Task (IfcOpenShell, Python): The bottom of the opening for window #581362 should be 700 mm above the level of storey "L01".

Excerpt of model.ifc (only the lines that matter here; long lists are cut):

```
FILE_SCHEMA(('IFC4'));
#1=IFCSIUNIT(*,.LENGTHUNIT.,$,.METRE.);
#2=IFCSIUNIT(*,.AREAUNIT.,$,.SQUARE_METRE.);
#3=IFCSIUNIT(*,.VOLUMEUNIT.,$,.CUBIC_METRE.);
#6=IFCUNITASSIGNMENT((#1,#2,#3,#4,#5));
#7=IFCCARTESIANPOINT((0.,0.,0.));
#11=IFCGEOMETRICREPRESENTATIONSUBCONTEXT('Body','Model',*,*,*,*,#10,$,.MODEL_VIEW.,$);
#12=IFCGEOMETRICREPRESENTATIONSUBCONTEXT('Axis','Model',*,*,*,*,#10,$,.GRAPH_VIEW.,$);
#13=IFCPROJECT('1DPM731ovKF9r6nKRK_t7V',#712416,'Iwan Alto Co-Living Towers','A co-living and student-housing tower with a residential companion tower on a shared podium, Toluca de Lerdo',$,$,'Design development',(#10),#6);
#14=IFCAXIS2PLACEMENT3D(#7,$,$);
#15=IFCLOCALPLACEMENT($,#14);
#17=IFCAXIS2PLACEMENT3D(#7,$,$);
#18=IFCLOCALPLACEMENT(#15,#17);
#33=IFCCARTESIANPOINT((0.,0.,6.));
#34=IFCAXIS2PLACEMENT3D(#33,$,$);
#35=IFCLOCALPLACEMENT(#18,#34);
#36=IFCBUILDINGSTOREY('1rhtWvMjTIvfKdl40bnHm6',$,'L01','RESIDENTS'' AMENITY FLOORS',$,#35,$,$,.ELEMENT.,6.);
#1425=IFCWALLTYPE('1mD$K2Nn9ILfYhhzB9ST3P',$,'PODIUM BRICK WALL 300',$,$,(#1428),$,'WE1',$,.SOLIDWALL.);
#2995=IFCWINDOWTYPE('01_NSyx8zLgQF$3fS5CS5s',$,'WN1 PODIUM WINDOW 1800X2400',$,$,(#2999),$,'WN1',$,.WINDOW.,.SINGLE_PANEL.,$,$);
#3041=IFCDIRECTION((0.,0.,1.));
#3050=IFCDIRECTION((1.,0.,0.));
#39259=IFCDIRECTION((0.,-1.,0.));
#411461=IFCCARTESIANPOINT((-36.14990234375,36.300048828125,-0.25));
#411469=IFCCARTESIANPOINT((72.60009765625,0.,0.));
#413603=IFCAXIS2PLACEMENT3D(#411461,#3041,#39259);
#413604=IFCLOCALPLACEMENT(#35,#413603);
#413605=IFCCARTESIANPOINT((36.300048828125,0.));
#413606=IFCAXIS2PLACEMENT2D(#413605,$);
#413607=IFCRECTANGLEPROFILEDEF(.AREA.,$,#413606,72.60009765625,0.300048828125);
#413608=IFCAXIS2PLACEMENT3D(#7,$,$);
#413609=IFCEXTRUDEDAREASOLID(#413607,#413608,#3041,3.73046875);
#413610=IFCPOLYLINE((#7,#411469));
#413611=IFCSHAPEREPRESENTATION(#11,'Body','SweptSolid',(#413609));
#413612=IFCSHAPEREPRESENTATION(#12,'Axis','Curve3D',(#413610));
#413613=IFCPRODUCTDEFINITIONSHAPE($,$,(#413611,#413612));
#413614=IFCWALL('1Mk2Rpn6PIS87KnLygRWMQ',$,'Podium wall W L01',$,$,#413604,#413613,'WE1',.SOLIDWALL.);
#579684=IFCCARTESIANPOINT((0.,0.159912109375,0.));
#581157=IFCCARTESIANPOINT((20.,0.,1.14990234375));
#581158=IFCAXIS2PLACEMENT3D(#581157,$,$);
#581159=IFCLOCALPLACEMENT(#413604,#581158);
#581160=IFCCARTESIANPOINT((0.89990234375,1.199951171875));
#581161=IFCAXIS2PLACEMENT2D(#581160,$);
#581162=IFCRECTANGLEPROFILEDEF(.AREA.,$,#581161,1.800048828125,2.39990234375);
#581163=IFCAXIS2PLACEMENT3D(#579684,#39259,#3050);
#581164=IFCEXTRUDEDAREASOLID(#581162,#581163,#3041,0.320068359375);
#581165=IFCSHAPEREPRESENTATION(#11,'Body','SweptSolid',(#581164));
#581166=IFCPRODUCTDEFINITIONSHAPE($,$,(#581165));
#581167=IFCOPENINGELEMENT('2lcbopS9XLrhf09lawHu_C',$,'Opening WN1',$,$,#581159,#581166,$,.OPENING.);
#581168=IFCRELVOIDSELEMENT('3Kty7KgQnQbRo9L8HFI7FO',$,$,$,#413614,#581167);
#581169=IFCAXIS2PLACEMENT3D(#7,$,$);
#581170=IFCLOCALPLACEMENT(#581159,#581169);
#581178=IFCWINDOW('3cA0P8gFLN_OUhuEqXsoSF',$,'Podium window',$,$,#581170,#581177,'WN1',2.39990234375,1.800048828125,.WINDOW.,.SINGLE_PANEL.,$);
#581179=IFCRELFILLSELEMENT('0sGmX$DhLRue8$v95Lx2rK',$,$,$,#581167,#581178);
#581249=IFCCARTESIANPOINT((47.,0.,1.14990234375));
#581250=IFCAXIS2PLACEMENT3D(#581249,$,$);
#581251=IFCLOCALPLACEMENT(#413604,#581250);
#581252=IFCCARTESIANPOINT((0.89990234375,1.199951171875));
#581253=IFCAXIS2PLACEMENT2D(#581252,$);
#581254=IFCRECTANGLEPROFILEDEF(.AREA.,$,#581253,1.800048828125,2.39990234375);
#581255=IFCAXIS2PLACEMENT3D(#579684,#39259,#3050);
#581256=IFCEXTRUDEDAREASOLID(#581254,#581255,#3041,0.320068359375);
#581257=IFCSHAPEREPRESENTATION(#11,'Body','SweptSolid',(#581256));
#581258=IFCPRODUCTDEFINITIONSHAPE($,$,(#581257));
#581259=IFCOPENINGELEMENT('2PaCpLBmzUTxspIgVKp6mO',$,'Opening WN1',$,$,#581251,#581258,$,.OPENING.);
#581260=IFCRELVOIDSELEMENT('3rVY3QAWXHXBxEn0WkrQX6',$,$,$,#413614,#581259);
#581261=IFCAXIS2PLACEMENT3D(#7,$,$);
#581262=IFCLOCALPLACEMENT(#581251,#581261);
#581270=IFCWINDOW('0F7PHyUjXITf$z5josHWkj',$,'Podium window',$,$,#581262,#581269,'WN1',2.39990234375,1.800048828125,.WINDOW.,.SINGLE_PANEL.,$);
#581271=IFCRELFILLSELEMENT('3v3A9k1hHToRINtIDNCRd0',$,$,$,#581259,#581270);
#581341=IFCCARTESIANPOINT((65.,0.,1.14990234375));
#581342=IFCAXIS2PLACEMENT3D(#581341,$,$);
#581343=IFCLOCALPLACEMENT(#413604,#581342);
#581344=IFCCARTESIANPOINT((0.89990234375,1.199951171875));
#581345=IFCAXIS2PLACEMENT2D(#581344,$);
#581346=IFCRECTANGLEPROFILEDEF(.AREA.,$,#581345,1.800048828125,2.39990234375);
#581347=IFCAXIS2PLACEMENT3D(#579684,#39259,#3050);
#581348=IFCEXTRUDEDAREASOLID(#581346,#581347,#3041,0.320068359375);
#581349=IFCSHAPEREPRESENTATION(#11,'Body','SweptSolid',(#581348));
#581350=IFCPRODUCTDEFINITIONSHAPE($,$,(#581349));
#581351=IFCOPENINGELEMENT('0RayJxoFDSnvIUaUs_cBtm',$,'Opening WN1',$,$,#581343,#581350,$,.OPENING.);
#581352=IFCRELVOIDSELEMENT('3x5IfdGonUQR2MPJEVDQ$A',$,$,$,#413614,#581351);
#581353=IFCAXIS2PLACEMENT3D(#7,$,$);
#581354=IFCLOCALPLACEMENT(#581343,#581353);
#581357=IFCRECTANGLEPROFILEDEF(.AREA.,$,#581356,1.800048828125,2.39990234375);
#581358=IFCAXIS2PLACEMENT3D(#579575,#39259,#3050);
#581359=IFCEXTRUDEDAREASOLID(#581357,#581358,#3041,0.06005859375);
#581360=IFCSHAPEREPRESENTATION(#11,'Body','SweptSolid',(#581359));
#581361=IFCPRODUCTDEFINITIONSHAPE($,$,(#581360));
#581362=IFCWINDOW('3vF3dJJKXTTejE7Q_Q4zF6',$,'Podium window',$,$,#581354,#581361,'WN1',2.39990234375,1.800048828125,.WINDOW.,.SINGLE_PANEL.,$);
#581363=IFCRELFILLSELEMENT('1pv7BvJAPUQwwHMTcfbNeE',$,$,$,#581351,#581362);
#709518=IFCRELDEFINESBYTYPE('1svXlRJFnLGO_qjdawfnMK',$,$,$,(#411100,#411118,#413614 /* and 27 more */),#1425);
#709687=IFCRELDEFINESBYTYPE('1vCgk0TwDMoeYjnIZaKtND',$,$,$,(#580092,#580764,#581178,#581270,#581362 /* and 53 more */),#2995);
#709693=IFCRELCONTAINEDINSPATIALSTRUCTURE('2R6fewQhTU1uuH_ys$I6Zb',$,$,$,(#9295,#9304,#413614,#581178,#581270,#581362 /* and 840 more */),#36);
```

```python
import numpy as np
import ifcopenshell
import ifcopenshell.api.geometry
import ifcopenshell.geom
import ifcopenshell.util.element
import ifcopenshell.util.placement
import ifcopenshell.util.shape
import ifcopenshell.util.unit

model = ifcopenshell.open("model.ifc")
unit_scale = ifcopenshell.util.unit.calculate_unit_scale(model)

window = model.by_guid("3vF3dJJKXTTejE7Q_Q4zF6")
opening = window.FillsVoids[0].RelatingOpeningElement
storey = ifcopenshell.util.element.get_container(window, ifc_class="IfcBuildingStorey")
level = ifcopenshell.util.placement.get_local_placement(storey.ObjectPlacement)[2, 3]

# The opening's origin need not be at the sill, so measure its lowest point.
shape = ifcopenshell.geom.create_shape(ifcopenshell.geom.settings(), opening)
bottom = ifcopenshell.util.shape.get_shape_bottom_elevation(shape, shape.geometry) / unit_scale
dz = level + 0.7 - bottom

shift = np.array([0.0, 0.0, dz])
# The window is placed relative to its opening, so it follows when the opening moves.
matrix = ifcopenshell.util.placement.get_local_placement(opening.ObjectPlacement)
matrix[:3, 3] += shift
ifcopenshell.api.geometry.edit_object_placement(
    model, product=opening, matrix=matrix, is_si=False, should_transform_children=True
)

print(f"moved by {dz * unit_scale:+.3f} m")

model.write("model_updated.ifc")
```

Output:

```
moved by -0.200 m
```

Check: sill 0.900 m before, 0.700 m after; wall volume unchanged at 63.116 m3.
